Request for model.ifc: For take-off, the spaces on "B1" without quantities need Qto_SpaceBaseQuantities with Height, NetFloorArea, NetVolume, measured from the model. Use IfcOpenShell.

First a look at what the model holds.

```python
import ifcopenshell
import ifcopenshell.util.element
import ifcopenshell.util.unit

model = ifcopenshell.open("model.ifc")
print(model.schema)
for unit_type in ("LENGTHUNIT", "AREAUNIT", "VOLUMEUNIT"):
    print(unit_type, ifcopenshell.util.unit.calculate_unit_scale(model, unit_type))
storey = next(s for s in model.by_type("IfcBuildingStorey") if s.Name == "B1")
spaces = [e for e in ifcopenshell.util.element.get_decomposition(storey) if e.is_a("IfcSpace")]
for e in sorted(spaces, key=lambda e: e.id()):
    print(e.id(), e.is_a(), e.Name, list(ifcopenshell.util.element.get_psets(e, qtos_only=True)), sep=" | ")
```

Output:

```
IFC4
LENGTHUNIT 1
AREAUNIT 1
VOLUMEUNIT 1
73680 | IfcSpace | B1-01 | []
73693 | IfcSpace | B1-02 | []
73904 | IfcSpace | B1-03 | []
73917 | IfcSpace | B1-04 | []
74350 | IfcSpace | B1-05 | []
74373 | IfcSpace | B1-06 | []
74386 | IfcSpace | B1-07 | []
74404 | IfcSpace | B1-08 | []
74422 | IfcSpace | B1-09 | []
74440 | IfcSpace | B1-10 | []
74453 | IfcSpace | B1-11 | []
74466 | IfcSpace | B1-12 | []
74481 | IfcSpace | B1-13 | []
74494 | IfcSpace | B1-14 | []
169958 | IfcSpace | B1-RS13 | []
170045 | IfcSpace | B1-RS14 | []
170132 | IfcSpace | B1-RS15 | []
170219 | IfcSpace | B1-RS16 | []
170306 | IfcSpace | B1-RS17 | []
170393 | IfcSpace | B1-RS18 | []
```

```python
import ifcopenshell
import ifcopenshell.api.pset
import ifcopenshell.geom
import ifcopenshell.util.element
import ifcopenshell.util.shape
import ifcopenshell.util.unit

model = ifcopenshell.open("model.ifc")
unit_scale = ifcopenshell.util.unit.calculate_unit_scale(model)
area_scale = ifcopenshell.util.unit.calculate_unit_scale(model, "AREAUNIT")
volume_scale = ifcopenshell.util.unit.calculate_unit_scale(model, "VOLUMEUNIT")
settings = ifcopenshell.geom.settings()

storey = next(s for s in model.by_type("IfcBuildingStorey") if s.Name == "B1")
spaces = [e for e in ifcopenshell.util.element.get_decomposition(storey) if e.is_a("IfcSpace")]

for e in sorted(spaces, key=lambda e: e.id()):
    if ifcopenshell.util.element.get_psets(e, qtos_only=True, should_inherit=False):
        continue
    # Geometry comes back in metres, in the element's own axes.
    shape = ifcopenshell.geom.create_shape(settings, e)
    values = {
        "Height": ifcopenshell.util.shape.get_z(shape.geometry) / unit_scale,
        "NetFloorArea": ifcopenshell.util.shape.get_footprint_area(shape.geometry) / area_scale,
        "NetVolume": ifcopenshell.util.shape.get_volume(shape.geometry) / volume_scale,
    }
    qto = ifcopenshell.api.pset.add_qto(model, product=e, name="Qto_SpaceBaseQuantities")
    ifcopenshell.api.pset.edit_qto(model, qto=qto, properties=values)
    print(e.id(), {k: round(v, 3) for k, v in values.items()})

model.write("model_rev.ifc")
```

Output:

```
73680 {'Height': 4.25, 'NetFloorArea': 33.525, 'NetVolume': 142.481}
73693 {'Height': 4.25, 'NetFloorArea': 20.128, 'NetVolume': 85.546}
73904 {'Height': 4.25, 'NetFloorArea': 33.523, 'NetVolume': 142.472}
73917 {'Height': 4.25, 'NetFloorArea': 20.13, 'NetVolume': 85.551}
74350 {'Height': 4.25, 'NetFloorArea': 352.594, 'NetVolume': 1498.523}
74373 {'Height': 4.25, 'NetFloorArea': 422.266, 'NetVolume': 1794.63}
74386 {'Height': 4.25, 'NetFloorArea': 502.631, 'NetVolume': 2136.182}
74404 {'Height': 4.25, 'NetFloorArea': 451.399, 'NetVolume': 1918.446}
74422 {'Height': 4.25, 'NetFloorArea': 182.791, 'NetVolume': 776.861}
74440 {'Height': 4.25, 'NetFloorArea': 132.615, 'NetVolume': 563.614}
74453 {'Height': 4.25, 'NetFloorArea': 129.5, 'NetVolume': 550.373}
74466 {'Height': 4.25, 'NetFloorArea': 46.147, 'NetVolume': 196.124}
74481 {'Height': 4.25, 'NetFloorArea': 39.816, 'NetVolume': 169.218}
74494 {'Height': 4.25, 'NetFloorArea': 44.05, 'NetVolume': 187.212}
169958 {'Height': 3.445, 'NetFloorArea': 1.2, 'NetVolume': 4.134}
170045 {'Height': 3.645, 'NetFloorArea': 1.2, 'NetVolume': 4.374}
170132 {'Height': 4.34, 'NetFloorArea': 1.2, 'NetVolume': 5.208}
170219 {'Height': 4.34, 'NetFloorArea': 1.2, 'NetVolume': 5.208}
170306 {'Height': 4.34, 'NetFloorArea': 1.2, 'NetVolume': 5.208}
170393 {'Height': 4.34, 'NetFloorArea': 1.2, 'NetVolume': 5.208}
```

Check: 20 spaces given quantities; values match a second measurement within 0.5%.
